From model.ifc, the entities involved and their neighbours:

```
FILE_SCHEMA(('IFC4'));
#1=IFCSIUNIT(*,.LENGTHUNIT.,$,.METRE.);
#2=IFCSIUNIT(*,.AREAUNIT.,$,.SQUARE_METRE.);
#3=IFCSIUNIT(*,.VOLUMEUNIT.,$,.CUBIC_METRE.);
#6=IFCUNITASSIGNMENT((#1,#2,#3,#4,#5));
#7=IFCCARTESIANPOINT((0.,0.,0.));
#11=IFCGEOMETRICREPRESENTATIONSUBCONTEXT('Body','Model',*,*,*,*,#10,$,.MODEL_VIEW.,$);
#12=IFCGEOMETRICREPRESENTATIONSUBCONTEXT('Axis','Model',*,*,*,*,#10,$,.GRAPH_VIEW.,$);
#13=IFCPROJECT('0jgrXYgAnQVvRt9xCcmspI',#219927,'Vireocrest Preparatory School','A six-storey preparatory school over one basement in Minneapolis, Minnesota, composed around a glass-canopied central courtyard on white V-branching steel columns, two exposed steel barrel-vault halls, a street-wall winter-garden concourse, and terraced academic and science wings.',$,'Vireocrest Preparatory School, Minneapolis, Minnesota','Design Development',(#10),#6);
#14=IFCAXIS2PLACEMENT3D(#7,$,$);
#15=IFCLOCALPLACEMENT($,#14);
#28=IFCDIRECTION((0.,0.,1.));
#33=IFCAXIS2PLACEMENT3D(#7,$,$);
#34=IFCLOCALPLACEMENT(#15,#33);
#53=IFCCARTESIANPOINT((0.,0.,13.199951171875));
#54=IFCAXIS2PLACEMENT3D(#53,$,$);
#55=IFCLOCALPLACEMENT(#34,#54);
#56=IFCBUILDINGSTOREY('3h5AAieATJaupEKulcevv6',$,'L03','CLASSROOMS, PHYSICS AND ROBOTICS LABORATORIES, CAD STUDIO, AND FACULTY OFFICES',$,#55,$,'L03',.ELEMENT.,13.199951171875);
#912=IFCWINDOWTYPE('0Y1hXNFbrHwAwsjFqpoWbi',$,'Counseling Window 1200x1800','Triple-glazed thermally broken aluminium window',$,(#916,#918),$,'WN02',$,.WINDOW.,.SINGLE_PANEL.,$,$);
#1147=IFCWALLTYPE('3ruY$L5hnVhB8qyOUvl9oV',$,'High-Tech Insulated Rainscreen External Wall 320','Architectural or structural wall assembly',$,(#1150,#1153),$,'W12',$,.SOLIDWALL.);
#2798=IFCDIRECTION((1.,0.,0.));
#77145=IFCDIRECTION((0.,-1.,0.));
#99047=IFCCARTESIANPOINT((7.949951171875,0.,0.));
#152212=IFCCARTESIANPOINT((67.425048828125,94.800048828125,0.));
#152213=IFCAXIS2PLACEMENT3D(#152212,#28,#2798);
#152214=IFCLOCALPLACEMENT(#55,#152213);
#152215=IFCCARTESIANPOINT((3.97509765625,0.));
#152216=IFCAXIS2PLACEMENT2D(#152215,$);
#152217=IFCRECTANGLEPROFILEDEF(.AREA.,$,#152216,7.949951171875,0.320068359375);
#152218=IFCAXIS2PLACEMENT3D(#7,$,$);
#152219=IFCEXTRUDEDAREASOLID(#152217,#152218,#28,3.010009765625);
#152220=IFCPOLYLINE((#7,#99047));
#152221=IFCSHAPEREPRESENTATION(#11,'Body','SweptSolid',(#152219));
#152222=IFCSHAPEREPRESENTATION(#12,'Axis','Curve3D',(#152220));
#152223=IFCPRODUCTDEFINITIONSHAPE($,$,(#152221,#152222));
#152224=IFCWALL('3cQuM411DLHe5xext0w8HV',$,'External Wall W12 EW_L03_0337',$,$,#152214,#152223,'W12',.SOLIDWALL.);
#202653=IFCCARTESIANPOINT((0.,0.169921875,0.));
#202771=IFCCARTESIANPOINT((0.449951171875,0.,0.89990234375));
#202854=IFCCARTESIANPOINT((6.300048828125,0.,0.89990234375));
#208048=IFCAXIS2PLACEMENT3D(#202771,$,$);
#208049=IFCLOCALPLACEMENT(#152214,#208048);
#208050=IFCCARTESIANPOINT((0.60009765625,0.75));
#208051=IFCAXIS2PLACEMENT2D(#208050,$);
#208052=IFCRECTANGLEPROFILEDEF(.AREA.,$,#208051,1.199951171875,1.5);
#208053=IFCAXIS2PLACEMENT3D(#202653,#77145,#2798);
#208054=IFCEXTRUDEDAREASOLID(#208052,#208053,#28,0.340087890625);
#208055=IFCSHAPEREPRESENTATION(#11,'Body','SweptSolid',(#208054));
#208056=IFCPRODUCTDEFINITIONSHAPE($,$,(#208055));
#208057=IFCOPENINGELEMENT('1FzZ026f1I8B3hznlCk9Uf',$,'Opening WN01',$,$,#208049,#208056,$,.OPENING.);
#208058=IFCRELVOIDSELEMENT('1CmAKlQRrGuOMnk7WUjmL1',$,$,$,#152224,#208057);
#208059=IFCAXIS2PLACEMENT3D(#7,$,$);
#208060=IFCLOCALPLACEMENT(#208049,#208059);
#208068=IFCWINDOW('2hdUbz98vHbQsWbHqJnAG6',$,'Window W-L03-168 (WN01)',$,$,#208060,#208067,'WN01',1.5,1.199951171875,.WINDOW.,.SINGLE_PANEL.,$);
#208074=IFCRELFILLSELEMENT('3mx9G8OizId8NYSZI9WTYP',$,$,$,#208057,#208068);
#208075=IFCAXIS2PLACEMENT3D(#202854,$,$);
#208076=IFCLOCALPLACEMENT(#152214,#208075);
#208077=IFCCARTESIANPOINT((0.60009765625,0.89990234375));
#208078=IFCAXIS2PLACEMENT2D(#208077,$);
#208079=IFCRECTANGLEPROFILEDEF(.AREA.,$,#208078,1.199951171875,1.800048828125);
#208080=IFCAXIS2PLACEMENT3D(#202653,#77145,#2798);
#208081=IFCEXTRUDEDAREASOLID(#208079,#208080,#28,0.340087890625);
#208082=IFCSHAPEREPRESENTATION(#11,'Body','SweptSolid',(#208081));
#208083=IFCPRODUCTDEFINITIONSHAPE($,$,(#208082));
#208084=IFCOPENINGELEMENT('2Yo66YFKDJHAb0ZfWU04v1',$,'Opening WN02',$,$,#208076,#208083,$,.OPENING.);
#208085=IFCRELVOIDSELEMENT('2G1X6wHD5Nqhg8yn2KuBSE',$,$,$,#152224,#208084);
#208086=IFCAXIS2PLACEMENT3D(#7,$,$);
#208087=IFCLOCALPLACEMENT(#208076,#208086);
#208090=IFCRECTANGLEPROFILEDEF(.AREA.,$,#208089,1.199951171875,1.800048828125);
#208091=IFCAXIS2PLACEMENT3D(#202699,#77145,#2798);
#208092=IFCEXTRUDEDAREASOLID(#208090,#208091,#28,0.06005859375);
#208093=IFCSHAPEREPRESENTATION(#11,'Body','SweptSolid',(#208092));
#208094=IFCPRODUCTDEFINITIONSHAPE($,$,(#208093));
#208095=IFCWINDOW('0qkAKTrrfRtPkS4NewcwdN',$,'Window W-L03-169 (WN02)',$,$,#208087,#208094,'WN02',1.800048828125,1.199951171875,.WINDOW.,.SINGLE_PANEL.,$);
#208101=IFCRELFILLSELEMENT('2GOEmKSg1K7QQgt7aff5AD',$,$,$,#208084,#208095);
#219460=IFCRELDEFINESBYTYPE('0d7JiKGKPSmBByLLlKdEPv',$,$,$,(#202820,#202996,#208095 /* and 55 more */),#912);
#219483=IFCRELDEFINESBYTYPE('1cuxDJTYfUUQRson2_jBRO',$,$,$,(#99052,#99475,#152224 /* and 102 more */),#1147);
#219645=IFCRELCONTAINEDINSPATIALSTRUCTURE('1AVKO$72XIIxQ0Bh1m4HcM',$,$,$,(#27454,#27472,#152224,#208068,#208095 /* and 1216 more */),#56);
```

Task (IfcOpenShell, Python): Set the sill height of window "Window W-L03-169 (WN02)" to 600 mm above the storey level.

```python
import numpy as np
import ifcopenshell
import ifcopenshell.api.geometry
import ifcopenshell.geom
import ifcopenshell.util.element
import ifcopenshell.util.placement
import ifcopenshell.util.shape
import ifcopenshell.util.unit

model = ifcopenshell.open("model.ifc")
unit_scale = ifcopenshell.util.unit.calculate_unit_scale(model)

window = model.by_id(208095)
opening = window.FillsVoids[0].RelatingOpeningElement
storey = ifcopenshell.util.element.get_container(window, ifc_class="IfcBuildingStorey")
level = ifcopenshell.util.placement.get_local_placement(storey.ObjectPlacement)[2, 3]

# The opening's origin need not be at the sill, so measure its lowest point.
shape = ifcopenshell.geom.create_shape(ifcopenshell.geom.settings(), opening)
bottom = ifcopenshell.util.shape.get_shape_bottom_elevation(shape, shape.geometry) / unit_scale
dz = level + 0.6 / unit_scale - bottom

shift = np.array([0.0, 0.0, dz])
# The window is placed relative to its opening, so it follows when the opening moves.
matrix = ifcopenshell.util.placement.get_local_placement(opening.ObjectPlacement)
matrix[:3, 3] += shift
ifcopenshell.api.geometry.edit_object_placement(
    model, product=opening, matrix=matrix, is_si=False, should_transform_children=True
)

print(f"moved by {dz * unit_scale:+.3f} m")

model.write("model_v2.ifc")
```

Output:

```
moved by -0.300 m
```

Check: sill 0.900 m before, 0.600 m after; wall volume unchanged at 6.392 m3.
